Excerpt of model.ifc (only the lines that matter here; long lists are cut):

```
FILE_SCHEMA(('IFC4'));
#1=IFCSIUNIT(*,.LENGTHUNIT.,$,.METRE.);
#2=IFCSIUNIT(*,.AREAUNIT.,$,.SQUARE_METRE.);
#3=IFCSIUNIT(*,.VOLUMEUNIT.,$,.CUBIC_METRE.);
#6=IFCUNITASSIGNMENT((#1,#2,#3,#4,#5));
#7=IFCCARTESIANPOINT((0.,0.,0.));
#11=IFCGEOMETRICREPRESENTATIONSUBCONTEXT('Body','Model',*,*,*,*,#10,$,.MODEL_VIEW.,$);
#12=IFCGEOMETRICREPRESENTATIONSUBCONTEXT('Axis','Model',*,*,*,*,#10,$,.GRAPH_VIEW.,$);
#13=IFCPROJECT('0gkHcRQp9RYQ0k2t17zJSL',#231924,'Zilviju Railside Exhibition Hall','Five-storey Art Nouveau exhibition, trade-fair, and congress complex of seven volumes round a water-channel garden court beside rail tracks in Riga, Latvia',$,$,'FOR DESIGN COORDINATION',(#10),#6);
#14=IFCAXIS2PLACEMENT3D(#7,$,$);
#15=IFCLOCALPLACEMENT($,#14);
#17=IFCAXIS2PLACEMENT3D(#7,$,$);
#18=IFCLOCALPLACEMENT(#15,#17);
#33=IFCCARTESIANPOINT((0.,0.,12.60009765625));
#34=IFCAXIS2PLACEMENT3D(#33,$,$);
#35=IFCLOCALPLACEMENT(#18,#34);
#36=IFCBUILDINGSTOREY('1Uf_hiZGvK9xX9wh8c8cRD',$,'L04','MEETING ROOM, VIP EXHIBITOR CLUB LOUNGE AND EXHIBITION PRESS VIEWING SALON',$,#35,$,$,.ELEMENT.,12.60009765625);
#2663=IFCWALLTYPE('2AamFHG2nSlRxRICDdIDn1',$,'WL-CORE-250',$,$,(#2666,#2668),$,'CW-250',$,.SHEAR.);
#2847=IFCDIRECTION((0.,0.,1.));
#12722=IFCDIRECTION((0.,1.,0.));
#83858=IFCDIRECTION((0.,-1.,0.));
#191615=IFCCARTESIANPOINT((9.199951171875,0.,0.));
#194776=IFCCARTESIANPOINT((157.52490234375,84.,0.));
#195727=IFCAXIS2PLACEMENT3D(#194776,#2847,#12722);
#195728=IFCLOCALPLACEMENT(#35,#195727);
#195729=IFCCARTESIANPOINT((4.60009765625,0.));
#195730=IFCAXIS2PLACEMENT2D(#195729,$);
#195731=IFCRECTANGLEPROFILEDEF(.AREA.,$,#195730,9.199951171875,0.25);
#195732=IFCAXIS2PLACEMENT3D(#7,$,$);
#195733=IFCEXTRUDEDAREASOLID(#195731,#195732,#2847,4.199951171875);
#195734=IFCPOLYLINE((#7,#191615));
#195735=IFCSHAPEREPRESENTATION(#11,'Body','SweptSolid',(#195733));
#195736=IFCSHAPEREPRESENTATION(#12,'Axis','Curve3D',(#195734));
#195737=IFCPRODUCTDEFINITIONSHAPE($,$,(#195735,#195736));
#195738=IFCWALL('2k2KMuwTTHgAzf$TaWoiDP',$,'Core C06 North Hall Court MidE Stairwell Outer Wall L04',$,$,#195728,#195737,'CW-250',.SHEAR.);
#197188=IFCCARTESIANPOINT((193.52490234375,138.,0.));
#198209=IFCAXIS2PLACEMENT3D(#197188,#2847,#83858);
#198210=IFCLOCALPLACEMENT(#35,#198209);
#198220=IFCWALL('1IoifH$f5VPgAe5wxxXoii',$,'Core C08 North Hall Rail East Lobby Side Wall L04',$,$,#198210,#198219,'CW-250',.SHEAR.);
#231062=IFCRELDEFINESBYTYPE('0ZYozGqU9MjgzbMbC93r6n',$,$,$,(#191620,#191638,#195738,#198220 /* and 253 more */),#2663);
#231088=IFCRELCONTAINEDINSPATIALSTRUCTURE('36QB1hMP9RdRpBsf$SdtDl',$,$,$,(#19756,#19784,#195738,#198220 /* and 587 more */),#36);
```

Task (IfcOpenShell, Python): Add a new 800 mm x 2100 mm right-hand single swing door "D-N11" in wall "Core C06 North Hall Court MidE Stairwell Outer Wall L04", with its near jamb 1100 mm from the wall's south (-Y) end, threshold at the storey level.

```python
import numpy as np
import ifcopenshell
import ifcopenshell.api.feature
import ifcopenshell.api.geometry
import ifcopenshell.api.root
import ifcopenshell.api.spatial
import ifcopenshell.geom
import ifcopenshell.util.element
import ifcopenshell.util.placement
import ifcopenshell.util.representation
import ifcopenshell.util.shape
import ifcopenshell.util.unit

model = ifcopenshell.open("model.ifc")
unit_scale = ifcopenshell.util.unit.calculate_unit_scale(model)
settings = ifcopenshell.geom.settings()


def volume(element):
    """Net volume in cubic metres, openings subtracted."""
    shape = ifcopenshell.geom.create_shape(settings, element)
    return ifcopenshell.util.shape.get_volume(shape.geometry)


wall = model.by_guid("2k2KMuwTTHgAzf$TaWoiDP")
storey = ifcopenshell.util.element.get_container(wall, ifc_class="IfcBuildingStorey")
context = ifcopenshell.util.representation.get_context(model, "Model", "Body", "MODEL_VIEW")
before = volume(wall)

width, height, from_end, sill = 0.8, 2.1, 1.1, 0.0  # metres

# The wall runs along its own X axis, and the end named is its -X end.
wall_shape = ifcopenshell.geom.create_shape(settings, wall)
x, y, z = ifcopenshell.util.shape.get_vertices(wall_shape.geometry).T
start = x.min() + from_end
face, thickness = float(y.min()), float(y.max() - y.min())
wall_matrix = ifcopenshell.util.placement.get_local_placement(wall.ObjectPlacement)
level = ifcopenshell.util.placement.get_local_placement(storey.ObjectPlacement)[2, 3]


def in_wall(x, y):
    """Placement at x, y metres in the wall's axes, at sill height."""
    matrix = wall_matrix.copy()
    matrix[:, 3] = wall_matrix @ np.array([x / unit_scale, y / unit_scale, 0.0, 1.0])
    matrix[2, 3] = level + sill / unit_scale
    return matrix


# Opening: a box that overshoots both wall faces by 50 mm.
opening = ifcopenshell.api.root.create_entity(model, ifc_class="IfcOpeningElement", predefined_type="OPENING")
box = ifcopenshell.api.geometry.add_wall_representation(
    model, context=context, length=width, height=height, thickness=thickness + 0.1
)
ifcopenshell.api.geometry.assign_representation(model, product=opening, representation=box)
ifcopenshell.api.geometry.edit_object_placement(model, product=opening, matrix=in_wall(start, face - 0.05), is_si=False)
ifcopenshell.api.feature.add_feature(model, feature=opening, element=wall)

door = ifcopenshell.api.root.create_entity(model, ifc_class="IfcDoor", name="D-N11", predefined_type="DOOR")
door.OverallWidth, door.OverallHeight = width / unit_scale, height / unit_scale
door.OperationType = "SINGLE_SWING_RIGHT"
body = ifcopenshell.api.geometry.add_door_representation(
    model,
    context=context,
    overall_width=door.OverallWidth,
    overall_height=door.OverallHeight,
    operation_type="SINGLE_SWING_RIGHT",
    lining_properties={"LiningDepth": thickness / unit_scale, "ThresholdDepth": thickness / unit_scale},
)
ifcopenshell.api.geometry.assign_representation(model, product=door, representation=body)
ifcopenshell.api.spatial.assign_container(model, products=[door], relating_structure=storey)
ifcopenshell.api.feature.add_filling(model, opening=opening, element=door)

# The lining spans the wall, so the door starts at the wall face.
ifcopenshell.api.geometry.edit_object_placement(model, product=door, matrix=in_wall(start, face), is_si=False)

after = volume(wall)

print(f"wall volume {before:.3f} -> {after:.3f} m3")

model.write("model-out.ifc")
```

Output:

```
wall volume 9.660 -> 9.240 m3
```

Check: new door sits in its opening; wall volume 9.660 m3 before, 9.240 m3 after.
